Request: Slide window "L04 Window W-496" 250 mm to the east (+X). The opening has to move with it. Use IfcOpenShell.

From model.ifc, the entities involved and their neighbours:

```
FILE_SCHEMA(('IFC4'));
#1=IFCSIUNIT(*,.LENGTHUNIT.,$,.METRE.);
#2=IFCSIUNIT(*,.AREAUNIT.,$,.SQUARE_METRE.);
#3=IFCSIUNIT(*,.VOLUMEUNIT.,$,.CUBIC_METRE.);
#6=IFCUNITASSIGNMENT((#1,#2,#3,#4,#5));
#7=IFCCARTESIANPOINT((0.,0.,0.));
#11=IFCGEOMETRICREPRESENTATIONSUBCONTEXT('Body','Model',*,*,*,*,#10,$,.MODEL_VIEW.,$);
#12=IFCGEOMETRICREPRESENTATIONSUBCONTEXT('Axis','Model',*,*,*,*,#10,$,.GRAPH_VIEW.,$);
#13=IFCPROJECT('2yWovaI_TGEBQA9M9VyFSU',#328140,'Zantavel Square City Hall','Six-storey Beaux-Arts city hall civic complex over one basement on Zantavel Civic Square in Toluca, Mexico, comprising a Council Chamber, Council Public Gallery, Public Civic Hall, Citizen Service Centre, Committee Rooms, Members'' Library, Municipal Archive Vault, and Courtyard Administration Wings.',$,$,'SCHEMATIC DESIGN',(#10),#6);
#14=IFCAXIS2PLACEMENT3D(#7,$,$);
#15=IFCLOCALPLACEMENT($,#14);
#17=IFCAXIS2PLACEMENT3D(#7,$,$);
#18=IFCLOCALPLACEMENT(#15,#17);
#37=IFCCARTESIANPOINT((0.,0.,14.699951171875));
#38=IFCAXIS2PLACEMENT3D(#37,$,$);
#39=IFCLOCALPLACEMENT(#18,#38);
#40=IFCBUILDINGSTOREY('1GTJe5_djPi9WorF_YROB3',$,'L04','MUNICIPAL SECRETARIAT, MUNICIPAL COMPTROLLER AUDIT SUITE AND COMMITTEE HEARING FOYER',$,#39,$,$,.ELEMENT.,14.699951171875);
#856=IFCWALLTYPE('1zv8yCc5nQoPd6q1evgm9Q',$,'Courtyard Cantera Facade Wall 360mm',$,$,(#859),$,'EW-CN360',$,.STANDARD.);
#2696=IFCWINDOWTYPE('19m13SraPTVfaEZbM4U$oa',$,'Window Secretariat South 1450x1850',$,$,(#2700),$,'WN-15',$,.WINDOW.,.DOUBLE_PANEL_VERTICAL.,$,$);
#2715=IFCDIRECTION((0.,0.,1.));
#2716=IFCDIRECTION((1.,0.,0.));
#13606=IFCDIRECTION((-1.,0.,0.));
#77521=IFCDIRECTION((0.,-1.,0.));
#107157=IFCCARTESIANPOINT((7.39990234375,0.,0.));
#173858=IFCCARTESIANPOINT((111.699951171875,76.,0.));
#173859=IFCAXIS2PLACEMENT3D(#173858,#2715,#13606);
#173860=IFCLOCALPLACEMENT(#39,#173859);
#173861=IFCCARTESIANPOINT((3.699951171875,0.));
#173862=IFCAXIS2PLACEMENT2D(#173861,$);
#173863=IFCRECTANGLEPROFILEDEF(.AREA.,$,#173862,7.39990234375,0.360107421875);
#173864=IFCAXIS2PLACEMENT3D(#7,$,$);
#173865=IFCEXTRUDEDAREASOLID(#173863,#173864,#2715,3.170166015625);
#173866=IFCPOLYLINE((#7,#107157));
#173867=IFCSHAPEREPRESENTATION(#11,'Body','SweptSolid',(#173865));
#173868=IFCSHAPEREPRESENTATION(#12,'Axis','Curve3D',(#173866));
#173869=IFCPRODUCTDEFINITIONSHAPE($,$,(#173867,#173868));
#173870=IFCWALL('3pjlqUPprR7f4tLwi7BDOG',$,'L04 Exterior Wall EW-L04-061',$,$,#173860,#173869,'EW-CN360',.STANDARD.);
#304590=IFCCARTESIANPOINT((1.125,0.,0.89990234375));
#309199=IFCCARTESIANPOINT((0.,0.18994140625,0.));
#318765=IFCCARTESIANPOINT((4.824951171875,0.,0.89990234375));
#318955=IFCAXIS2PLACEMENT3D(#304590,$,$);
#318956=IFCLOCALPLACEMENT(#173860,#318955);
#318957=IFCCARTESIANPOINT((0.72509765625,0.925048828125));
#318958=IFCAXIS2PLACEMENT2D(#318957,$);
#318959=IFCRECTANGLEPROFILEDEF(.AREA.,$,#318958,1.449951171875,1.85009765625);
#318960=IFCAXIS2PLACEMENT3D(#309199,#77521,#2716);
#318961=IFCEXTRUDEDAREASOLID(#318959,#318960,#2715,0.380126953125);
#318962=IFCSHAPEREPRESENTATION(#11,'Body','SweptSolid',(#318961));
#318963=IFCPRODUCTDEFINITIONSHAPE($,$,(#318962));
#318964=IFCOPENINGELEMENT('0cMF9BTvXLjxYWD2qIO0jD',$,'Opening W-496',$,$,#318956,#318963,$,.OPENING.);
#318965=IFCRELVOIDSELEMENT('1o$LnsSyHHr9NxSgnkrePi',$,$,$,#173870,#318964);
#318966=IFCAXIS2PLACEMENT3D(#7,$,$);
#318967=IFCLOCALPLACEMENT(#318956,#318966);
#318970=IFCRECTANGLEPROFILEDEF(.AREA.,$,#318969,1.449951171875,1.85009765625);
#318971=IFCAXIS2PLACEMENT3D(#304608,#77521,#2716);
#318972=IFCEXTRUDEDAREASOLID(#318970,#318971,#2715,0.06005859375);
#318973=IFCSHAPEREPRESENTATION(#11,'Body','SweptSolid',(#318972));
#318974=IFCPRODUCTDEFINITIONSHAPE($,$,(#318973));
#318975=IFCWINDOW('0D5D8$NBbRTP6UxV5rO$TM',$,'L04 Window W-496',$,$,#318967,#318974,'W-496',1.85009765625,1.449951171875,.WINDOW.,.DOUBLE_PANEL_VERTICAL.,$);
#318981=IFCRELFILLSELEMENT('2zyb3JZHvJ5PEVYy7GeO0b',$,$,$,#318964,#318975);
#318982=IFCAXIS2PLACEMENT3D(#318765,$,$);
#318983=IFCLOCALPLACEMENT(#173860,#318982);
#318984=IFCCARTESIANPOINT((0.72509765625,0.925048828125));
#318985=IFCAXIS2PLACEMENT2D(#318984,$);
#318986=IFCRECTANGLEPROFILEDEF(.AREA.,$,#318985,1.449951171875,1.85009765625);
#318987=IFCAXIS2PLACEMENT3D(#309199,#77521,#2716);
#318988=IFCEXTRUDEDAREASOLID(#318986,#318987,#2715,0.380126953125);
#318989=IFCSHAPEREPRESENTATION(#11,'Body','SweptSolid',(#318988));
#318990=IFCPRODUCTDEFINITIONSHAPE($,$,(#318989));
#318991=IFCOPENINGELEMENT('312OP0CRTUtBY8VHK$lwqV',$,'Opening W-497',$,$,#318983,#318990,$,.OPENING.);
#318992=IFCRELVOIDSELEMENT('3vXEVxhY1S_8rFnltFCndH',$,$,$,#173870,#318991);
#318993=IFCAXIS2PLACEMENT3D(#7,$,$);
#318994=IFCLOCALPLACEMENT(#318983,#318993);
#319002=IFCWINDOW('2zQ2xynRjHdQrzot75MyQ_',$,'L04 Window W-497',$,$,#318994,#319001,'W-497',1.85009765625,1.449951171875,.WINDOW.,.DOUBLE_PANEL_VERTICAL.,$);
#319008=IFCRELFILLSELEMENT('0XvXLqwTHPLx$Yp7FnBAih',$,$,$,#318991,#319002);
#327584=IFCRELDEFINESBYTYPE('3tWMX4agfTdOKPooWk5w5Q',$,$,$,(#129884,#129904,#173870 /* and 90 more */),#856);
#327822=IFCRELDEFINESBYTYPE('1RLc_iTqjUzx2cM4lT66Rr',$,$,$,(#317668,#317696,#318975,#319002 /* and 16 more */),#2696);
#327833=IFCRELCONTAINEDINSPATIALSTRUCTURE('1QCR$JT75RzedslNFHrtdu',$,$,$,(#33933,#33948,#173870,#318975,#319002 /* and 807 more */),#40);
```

```python
import ifcopenshell
import ifcopenshell.api.geometry
import ifcopenshell.util.placement
import ifcopenshell.util.unit

model = ifcopenshell.open("model.ifc")
unit_scale = ifcopenshell.util.unit.calculate_unit_scale(model)

window = model.by_id(318975)
opening = window.FillsVoids[0].RelatingOpeningElement
wall = opening.VoidsElements[0].RelatingBuildingElement

wall_matrix = ifcopenshell.util.placement.get_local_placement(wall.ObjectPlacement)
shift = wall_matrix[:3, 0] * -0.25 / unit_scale
before = ifcopenshell.util.placement.get_local_placement(window.ObjectPlacement)[:3, 3].copy()

# The window is placed relative to its opening, so it follows when the opening moves.
matrix = ifcopenshell.util.placement.get_local_placement(opening.ObjectPlacement)
matrix[:3, 3] += shift
ifcopenshell.api.geometry.edit_object_placement(
    model, product=opening, matrix=matrix, is_si=False, should_transform_children=True
)

after = ifcopenshell.util.placement.get_local_placement(window.ObjectPlacement)[:3, 3]
print("window moved by", (after - before).round(3) + 0.0)

model.write("model_updated.ifc")
```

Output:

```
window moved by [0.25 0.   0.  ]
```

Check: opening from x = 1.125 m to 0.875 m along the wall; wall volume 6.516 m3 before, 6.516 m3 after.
